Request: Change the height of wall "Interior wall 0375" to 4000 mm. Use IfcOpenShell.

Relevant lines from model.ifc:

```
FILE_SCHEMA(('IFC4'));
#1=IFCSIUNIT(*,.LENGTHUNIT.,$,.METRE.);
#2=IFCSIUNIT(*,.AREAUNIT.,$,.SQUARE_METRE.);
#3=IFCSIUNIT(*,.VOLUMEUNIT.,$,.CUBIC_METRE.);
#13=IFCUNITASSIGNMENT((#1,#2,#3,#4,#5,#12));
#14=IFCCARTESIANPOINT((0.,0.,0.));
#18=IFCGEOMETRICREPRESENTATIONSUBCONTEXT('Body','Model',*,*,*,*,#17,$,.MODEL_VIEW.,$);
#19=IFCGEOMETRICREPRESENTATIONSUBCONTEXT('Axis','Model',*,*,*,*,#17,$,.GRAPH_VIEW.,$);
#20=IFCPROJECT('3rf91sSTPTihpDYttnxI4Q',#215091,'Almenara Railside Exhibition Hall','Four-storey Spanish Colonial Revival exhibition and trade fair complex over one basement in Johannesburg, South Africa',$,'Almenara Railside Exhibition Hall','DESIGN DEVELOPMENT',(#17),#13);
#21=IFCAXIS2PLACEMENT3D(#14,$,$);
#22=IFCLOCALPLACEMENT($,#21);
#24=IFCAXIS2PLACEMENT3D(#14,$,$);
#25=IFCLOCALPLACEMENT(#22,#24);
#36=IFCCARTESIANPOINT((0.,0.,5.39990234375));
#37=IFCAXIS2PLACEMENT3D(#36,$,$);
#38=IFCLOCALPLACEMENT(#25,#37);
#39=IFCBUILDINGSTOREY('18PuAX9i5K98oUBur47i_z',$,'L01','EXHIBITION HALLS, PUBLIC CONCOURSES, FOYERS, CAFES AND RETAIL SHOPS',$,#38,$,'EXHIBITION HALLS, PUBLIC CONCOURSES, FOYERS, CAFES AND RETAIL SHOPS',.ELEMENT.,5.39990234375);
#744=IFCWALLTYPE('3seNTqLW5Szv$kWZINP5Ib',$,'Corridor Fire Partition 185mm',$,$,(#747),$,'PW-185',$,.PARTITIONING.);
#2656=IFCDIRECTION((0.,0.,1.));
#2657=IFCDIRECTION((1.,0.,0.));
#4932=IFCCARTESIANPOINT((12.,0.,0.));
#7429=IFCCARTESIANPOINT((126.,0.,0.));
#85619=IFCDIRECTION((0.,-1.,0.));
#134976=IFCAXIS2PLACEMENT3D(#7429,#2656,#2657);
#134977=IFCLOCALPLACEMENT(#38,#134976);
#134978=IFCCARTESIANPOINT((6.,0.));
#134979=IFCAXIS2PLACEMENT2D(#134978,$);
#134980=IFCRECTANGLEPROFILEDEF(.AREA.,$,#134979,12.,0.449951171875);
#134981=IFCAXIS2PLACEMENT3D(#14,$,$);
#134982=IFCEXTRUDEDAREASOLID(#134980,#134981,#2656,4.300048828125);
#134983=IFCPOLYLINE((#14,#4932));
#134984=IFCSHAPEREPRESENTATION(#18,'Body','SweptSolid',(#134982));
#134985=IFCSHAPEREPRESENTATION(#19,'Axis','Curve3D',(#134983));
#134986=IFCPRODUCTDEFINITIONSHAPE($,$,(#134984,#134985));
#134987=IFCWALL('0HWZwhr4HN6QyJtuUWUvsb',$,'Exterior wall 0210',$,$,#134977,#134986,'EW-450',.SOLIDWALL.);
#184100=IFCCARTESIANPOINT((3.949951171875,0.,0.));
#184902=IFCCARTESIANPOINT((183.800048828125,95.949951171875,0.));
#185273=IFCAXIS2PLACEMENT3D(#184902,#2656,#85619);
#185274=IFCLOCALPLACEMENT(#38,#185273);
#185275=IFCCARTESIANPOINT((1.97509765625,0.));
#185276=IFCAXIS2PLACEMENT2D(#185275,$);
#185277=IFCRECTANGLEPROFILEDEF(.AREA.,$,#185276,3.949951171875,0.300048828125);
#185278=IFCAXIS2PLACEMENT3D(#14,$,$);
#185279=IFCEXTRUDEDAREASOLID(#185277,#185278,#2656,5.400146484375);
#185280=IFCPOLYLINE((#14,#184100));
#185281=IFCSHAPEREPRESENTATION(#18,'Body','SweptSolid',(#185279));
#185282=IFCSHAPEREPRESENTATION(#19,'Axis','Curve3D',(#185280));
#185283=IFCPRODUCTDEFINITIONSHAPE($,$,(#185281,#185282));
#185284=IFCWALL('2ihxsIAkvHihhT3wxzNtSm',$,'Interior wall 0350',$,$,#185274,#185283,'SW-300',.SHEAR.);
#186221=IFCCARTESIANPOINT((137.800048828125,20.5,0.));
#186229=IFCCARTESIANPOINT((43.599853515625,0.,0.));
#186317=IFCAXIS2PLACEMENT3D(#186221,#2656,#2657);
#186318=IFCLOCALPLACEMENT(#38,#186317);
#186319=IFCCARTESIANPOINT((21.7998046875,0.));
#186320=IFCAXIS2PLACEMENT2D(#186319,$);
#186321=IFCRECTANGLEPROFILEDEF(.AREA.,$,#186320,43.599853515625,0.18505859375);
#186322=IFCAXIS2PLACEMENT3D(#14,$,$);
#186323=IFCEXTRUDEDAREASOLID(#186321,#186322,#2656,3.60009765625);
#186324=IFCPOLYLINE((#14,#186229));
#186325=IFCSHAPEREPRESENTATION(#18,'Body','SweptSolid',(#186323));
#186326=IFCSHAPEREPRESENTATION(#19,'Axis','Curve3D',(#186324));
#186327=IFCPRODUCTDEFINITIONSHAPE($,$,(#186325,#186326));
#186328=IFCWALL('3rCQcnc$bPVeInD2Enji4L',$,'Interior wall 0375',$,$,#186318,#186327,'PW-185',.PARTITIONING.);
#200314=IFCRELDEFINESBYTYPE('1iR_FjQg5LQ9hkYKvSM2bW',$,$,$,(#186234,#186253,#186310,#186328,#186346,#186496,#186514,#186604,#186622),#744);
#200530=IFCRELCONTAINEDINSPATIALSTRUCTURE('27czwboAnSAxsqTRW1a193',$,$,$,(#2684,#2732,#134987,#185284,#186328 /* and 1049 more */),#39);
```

```python
import ifcopenshell
import ifcopenshell.geom
import ifcopenshell.util.representation
import ifcopenshell.util.shape

model = ifcopenshell.open("model.ifc")
settings = ifcopenshell.geom.settings()


def volume(element):
    """Net volume in cubic metres, openings subtracted."""
    shape = ifcopenshell.geom.create_shape(settings, element)
    return ifcopenshell.util.shape.get_volume(shape.geometry)


wall = model.by_guid("3rCQcnc$bPVeInD2Enji4L")
before = volume(wall)

body = ifcopenshell.util.representation.get_representation(wall, "Model", "Body")
solid = body.Items[0]
old_height = solid.Depth
solid.Depth = 4.0
after = volume(wall)

print(f"height {old_height:g} -> {solid.Depth:g}, volume {before:.3f} -> {after:.3f} m3")

model.write("model-out.ifc")
```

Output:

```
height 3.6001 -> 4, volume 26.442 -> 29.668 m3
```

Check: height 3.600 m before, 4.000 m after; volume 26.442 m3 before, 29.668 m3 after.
